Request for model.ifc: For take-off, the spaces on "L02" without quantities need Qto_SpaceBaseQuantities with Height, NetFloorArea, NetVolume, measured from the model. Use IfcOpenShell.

First a look at what the model holds.

```python
import ifcopenshell
import ifcopenshell.util.element
import ifcopenshell.util.unit

model = ifcopenshell.open("model.ifc")
print(model.schema)
for unit_type in ("LENGTHUNIT", "AREAUNIT", "VOLUMEUNIT"):
    print(unit_type, ifcopenshell.util.unit.calculate_unit_scale(model, unit_type))
storey = next(s for s in model.by_type("IfcBuildingStorey") if s.Name == "L02")
spaces = [e for e in ifcopenshell.util.element.get_decomposition(storey) if e.is_a("IfcSpace")]
for e in sorted(spaces, key=lambda e: e.id()):
    print(e.id(), e.is_a(), e.Name, list(ifcopenshell.util.element.get_psets(e, qtos_only=True)), sep=" | ")
```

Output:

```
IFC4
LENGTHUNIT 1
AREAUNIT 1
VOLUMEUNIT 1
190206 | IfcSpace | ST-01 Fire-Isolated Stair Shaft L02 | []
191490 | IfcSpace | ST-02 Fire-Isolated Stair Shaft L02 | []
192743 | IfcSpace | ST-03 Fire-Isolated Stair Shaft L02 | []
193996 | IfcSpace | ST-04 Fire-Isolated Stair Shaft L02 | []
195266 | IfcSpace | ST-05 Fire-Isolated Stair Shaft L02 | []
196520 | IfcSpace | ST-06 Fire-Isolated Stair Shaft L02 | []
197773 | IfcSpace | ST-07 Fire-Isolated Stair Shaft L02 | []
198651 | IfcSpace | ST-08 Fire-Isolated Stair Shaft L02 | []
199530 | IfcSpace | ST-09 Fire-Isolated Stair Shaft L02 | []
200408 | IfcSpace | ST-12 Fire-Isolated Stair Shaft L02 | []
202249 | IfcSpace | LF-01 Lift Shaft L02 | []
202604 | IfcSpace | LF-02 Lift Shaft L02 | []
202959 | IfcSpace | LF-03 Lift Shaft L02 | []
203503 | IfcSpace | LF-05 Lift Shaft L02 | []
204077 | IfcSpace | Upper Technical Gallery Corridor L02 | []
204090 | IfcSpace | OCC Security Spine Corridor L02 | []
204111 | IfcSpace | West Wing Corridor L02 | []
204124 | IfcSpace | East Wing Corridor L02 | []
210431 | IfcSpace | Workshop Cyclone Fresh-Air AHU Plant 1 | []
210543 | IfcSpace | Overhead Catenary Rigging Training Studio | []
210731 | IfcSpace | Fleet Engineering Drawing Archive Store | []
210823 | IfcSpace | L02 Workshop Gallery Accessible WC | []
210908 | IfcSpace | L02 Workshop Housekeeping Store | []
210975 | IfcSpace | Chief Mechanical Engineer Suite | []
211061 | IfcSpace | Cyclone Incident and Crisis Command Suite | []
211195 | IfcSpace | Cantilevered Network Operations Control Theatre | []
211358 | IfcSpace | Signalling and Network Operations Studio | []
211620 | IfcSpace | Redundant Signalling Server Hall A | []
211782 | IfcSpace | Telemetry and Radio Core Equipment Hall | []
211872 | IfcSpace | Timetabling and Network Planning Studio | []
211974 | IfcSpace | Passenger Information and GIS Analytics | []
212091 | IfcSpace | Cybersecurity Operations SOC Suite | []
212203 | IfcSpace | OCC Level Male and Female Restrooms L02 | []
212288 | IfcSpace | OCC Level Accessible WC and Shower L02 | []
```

```python
import ifcopenshell
import ifcopenshell.api.pset
import ifcopenshell.geom
import ifcopenshell.util.element
import ifcopenshell.util.shape
import ifcopenshell.util.unit

model = ifcopenshell.open("model.ifc")
unit_scale = ifcopenshell.util.unit.calculate_unit_scale(model)
area_scale = ifcopenshell.util.unit.calculate_unit_scale(model, "AREAUNIT")
volume_scale = ifcopenshell.util.unit.calculate_unit_scale(model, "VOLUMEUNIT")
settings = ifcopenshell.geom.settings()

storey = next(s for s in model.by_type("IfcBuildingStorey") if s.Name == "L02")
spaces = [e for e in ifcopenshell.util.element.get_decomposition(storey) if e.is_a("IfcSpace")]

for e in sorted(spaces, key=lambda e: e.id()):
    if ifcopenshell.util.element.get_psets(e, qtos_only=True, should_inherit=False):
        continue
    # Geometry comes back in metres, in the element's own axes.
    shape = ifcopenshell.geom.create_shape(settings, e)
    values = {
        "Height": ifcopenshell.util.shape.get_z(shape.geometry) / unit_scale,
        "NetFloorArea": ifcopenshell.util.shape.get_footprint_area(shape.geometry) / area_scale,
        "NetVolume": ifcopenshell.util.shape.get_volume(shape.geometry) / volume_scale,
    }
    qto = ifcopenshell.api.pset.add_qto(model, product=e, name="Qto_SpaceBaseQuantities")
    ifcopenshell.api.pset.edit_qto(model, qto=qto, properties=values)
    print(e.id(), {k: round(v, 3) for k, v in values.items()})

model.write("model_v2.ifc")
```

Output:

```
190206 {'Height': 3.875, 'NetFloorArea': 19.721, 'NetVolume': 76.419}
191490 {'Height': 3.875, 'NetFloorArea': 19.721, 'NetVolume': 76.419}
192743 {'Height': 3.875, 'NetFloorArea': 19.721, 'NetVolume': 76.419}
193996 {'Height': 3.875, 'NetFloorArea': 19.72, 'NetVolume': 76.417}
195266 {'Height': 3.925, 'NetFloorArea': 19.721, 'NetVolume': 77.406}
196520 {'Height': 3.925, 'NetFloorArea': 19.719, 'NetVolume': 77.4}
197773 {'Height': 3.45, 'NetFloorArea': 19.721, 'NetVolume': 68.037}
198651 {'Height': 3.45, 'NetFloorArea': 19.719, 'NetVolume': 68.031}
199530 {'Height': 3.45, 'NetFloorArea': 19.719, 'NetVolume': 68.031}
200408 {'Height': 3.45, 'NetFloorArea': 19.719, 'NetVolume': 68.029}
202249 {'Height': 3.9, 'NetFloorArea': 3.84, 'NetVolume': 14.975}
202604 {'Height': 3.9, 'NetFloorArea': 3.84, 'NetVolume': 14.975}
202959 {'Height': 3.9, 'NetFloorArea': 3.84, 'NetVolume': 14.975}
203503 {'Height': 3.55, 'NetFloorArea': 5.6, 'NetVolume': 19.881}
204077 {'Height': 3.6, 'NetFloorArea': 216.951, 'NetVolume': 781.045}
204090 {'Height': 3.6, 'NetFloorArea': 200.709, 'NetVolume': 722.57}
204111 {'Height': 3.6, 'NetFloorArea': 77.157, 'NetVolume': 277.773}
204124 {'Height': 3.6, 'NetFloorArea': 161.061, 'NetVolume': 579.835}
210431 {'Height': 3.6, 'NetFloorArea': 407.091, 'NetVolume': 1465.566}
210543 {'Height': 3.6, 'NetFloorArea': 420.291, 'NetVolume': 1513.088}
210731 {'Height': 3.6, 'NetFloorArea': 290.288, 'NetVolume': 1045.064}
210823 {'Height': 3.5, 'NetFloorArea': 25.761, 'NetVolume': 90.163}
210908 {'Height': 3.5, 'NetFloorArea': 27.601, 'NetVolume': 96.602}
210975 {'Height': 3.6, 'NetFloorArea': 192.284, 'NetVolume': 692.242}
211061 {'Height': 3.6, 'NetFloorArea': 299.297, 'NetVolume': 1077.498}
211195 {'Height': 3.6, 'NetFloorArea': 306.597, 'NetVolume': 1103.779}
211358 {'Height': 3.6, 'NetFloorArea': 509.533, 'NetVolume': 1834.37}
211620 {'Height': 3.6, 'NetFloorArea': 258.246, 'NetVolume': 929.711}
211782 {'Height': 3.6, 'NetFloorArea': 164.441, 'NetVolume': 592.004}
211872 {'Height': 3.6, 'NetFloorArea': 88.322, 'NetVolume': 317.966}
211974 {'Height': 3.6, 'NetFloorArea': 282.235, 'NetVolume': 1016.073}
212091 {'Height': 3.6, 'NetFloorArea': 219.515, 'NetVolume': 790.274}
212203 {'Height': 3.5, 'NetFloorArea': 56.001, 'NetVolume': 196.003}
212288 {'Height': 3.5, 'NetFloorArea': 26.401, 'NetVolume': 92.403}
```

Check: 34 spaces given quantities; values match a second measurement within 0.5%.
